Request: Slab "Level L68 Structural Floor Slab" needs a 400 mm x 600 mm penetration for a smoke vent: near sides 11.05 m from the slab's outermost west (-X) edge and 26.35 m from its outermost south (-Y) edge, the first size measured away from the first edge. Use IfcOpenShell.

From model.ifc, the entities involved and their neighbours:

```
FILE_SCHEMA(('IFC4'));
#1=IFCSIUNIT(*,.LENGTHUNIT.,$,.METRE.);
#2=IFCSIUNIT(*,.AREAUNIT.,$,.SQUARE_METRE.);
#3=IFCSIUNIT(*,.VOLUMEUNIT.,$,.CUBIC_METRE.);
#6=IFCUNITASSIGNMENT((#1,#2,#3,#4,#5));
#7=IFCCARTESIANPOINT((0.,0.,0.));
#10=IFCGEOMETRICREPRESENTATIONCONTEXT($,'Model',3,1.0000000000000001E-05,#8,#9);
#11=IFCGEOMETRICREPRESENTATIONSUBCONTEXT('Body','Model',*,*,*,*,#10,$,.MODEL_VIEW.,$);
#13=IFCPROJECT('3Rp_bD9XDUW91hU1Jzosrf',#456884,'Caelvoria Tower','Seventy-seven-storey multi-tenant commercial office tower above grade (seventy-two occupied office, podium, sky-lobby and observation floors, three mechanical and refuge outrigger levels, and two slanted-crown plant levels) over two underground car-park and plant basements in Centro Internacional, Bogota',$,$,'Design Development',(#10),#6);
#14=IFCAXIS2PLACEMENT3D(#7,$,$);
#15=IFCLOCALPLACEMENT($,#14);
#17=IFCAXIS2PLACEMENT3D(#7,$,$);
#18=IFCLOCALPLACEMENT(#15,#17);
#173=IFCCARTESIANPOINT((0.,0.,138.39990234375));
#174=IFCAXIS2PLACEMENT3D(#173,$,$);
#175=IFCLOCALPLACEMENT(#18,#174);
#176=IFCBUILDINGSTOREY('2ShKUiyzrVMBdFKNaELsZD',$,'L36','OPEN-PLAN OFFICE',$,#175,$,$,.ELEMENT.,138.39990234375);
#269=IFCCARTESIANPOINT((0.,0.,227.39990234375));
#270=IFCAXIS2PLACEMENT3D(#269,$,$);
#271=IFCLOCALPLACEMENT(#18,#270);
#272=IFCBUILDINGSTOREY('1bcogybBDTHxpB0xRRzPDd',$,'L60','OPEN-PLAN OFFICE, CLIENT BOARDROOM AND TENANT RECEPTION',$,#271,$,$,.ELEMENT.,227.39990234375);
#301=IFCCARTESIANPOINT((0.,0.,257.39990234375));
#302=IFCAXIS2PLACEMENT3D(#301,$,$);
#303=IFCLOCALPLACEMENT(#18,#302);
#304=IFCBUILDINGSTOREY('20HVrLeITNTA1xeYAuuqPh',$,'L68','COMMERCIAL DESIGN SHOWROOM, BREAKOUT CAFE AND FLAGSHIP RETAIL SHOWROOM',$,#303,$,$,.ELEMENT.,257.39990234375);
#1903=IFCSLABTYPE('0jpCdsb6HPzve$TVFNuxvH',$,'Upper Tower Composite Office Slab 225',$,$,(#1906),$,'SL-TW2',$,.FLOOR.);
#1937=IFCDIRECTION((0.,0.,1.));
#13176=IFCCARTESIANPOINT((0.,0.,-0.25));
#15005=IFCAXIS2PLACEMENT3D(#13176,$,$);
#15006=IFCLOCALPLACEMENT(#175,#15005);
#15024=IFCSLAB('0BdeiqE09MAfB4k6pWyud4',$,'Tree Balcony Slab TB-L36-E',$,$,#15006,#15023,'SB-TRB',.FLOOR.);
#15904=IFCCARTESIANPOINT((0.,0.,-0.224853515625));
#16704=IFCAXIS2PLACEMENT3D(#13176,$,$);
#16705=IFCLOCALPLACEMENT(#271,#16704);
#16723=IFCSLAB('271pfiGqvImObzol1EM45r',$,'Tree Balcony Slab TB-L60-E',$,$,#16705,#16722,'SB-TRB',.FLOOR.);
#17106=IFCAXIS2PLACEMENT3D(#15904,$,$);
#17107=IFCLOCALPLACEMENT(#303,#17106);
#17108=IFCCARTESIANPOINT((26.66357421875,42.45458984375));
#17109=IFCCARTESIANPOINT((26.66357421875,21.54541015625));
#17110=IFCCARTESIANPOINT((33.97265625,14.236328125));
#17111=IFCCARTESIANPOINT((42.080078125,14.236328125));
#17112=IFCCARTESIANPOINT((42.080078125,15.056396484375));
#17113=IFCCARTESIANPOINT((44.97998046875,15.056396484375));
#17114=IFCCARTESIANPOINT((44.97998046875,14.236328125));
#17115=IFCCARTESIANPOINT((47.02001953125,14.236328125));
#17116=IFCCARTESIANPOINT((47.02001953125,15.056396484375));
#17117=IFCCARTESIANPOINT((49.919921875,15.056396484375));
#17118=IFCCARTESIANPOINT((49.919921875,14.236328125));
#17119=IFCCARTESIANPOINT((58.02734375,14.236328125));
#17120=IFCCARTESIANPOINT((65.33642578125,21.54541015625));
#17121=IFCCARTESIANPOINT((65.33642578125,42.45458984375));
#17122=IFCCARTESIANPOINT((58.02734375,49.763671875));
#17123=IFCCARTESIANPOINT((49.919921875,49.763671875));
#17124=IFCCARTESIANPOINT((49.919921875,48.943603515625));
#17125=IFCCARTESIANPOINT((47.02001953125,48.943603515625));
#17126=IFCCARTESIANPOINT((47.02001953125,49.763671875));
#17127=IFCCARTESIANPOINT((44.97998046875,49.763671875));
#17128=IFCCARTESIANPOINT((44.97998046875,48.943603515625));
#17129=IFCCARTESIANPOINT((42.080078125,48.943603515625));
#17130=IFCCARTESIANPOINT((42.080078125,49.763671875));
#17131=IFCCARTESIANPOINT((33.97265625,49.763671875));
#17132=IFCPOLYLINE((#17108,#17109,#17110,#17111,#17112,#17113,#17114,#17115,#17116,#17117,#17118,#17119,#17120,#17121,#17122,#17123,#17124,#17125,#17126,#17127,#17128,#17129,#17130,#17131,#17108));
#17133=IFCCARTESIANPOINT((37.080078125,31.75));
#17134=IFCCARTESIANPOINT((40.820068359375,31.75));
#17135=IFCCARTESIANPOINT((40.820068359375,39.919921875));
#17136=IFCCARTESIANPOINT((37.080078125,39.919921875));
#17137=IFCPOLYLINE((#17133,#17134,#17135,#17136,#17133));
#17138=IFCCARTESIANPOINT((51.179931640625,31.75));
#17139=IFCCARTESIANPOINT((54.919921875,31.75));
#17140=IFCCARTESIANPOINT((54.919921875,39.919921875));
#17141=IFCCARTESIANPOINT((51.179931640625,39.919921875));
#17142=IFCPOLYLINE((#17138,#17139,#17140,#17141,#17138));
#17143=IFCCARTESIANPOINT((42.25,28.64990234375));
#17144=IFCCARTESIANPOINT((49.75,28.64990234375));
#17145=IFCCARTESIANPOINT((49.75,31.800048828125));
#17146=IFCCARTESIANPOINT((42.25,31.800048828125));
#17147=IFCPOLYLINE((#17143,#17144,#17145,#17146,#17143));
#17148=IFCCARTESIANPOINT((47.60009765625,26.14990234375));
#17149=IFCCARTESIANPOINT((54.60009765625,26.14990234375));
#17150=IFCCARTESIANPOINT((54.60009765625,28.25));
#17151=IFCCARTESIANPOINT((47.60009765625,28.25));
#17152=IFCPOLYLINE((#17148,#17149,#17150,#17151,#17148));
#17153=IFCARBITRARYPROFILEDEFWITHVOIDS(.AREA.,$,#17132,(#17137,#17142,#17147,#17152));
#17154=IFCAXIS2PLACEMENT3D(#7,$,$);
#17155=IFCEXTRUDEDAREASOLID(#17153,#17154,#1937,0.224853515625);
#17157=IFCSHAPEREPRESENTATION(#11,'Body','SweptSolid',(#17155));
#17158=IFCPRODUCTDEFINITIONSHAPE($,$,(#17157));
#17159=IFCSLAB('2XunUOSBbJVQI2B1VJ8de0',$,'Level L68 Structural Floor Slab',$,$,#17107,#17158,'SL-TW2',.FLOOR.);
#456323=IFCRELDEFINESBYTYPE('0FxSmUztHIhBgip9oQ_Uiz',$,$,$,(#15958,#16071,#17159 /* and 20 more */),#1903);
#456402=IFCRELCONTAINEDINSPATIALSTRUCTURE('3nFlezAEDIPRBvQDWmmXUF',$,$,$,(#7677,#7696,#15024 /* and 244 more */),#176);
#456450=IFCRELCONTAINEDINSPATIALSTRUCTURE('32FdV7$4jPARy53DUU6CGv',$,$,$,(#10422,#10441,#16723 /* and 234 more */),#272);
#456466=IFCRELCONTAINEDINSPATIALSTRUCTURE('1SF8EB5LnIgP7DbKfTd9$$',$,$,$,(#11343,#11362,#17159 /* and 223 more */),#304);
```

```python
import numpy as np
import ifcopenshell
import ifcopenshell.api.feature
import ifcopenshell.api.geometry
import ifcopenshell.api.root
import ifcopenshell.geom
import ifcopenshell.util.placement
import ifcopenshell.util.representation
import ifcopenshell.util.shape
import ifcopenshell.util.unit

model = ifcopenshell.open("model.ifc")
unit_scale = ifcopenshell.util.unit.calculate_unit_scale(model)
settings = ifcopenshell.geom.settings()


def volume(element):
    """Net volume in cubic metres, openings subtracted."""
    shape = ifcopenshell.geom.create_shape(settings, element)
    return ifcopenshell.util.shape.get_volume(shape.geometry)


slab = model.by_guid("2XunUOSBbJVQI2B1VJ8de0")
before = volume(slab)

# Extent in the slab's own axes, in metres. The edges named are its -X and -Y sides.
slab_shape = ifcopenshell.geom.create_shape(settings, slab)
vertices = ifcopenshell.util.shape.get_vertices(slab_shape.geometry)
x_min, y_min, bottom = vertices.min(axis=0)
top = vertices[:, 2].max()

opening = ifcopenshell.api.root.create_entity(model, ifc_class="IfcOpeningElement", name="Smoke vent opening", predefined_type="OPENING")
context = ifcopenshell.util.representation.get_context(model, "Model", "Body", "MODEL_VIEW")
width, depth = 0.4, 0.6
outline = [(0.0, 0.0), (width, 0.0), (width, depth), (0.0, depth), (0.0, 0.0)]
# Overshoot both faces by 50 mm so the cut is clean.
shape = ifcopenshell.api.geometry.add_slab_representation(
    model, context=context, depth=top - bottom + 0.1, polyline=outline
)
ifcopenshell.api.geometry.assign_representation(model, product=opening, representation=shape)

matrix = ifcopenshell.util.placement.get_local_placement(slab.ObjectPlacement)
matrix[:, 3] = matrix @ np.append(np.array([x_min + 11.05, y_min + 26.35, bottom - 0.05]) / unit_scale, 1.0)
ifcopenshell.api.geometry.edit_object_placement(model, product=opening, matrix=matrix, is_si=False)
ifcopenshell.api.feature.add_feature(model, feature=opening, element=slab)

after = volume(slab)

print(f"slab volume {before:.3f} -> {after:.3f} m3")

model.write("model_edited.ifc")
```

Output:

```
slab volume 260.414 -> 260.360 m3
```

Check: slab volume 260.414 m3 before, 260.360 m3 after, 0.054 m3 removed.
